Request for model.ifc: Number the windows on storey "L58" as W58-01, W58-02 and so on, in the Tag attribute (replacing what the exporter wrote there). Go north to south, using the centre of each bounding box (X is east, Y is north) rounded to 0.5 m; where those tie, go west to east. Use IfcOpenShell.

First a look at what the model holds.

```python
import ifcopenshell
import ifcopenshell.util.element
import ifcopenshell.util.placement

model = ifcopenshell.open("model.ifc")
print(model.schema)
storey = next(s for s in model.by_type("IfcBuildingStorey") if s.Name == "L58")
windows = [e for e in ifcopenshell.util.element.get_decomposition(storey) if e.is_a("IfcWindow")]
for e in sorted(windows, key=lambda e: e.id()):
    origin = ifcopenshell.util.placement.get_local_placement(e.ObjectPlacement)[:3, 3]
    print(e.id(), e.Tag, e.Name, origin.round(2) + 0.0, sep=" | ")
```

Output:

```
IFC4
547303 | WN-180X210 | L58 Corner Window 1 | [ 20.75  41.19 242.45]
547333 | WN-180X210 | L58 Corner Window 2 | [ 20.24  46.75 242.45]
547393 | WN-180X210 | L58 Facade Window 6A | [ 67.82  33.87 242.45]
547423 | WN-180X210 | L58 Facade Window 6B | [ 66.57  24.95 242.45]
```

```python
import ifcopenshell
import ifcopenshell.geom
import ifcopenshell.util.element
import ifcopenshell.util.shape

model = ifcopenshell.open("model.ifc")
settings = ifcopenshell.geom.settings()
settings.set("use-world-coords", True)


def centre(element):
    shape = ifcopenshell.geom.create_shape(settings, element)
    return ifcopenshell.util.shape.get_bbox_centroid(shape.geometry)


storey = next(s for s in model.by_type("IfcBuildingStorey") if s.Name == "L58")
windows = [e for e in ifcopenshell.util.element.get_decomposition(storey) if e.is_a("IfcWindow")]

# Insertion points can sit at a corner or the storey origin, so sort by the geometry (in metres).
centres = {e: centre(e) for e in windows}
windows.sort(key=lambda e: (-round(centres[e][1] / 0.5), centres[e][0]))

for i, e in enumerate(windows, start=1):
    number = f"W58-{i:02d}"
    e.Tag = number
    print(e.id(), number)

model.write("model_v2.ifc")
```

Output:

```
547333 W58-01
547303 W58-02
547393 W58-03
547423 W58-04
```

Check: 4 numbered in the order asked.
